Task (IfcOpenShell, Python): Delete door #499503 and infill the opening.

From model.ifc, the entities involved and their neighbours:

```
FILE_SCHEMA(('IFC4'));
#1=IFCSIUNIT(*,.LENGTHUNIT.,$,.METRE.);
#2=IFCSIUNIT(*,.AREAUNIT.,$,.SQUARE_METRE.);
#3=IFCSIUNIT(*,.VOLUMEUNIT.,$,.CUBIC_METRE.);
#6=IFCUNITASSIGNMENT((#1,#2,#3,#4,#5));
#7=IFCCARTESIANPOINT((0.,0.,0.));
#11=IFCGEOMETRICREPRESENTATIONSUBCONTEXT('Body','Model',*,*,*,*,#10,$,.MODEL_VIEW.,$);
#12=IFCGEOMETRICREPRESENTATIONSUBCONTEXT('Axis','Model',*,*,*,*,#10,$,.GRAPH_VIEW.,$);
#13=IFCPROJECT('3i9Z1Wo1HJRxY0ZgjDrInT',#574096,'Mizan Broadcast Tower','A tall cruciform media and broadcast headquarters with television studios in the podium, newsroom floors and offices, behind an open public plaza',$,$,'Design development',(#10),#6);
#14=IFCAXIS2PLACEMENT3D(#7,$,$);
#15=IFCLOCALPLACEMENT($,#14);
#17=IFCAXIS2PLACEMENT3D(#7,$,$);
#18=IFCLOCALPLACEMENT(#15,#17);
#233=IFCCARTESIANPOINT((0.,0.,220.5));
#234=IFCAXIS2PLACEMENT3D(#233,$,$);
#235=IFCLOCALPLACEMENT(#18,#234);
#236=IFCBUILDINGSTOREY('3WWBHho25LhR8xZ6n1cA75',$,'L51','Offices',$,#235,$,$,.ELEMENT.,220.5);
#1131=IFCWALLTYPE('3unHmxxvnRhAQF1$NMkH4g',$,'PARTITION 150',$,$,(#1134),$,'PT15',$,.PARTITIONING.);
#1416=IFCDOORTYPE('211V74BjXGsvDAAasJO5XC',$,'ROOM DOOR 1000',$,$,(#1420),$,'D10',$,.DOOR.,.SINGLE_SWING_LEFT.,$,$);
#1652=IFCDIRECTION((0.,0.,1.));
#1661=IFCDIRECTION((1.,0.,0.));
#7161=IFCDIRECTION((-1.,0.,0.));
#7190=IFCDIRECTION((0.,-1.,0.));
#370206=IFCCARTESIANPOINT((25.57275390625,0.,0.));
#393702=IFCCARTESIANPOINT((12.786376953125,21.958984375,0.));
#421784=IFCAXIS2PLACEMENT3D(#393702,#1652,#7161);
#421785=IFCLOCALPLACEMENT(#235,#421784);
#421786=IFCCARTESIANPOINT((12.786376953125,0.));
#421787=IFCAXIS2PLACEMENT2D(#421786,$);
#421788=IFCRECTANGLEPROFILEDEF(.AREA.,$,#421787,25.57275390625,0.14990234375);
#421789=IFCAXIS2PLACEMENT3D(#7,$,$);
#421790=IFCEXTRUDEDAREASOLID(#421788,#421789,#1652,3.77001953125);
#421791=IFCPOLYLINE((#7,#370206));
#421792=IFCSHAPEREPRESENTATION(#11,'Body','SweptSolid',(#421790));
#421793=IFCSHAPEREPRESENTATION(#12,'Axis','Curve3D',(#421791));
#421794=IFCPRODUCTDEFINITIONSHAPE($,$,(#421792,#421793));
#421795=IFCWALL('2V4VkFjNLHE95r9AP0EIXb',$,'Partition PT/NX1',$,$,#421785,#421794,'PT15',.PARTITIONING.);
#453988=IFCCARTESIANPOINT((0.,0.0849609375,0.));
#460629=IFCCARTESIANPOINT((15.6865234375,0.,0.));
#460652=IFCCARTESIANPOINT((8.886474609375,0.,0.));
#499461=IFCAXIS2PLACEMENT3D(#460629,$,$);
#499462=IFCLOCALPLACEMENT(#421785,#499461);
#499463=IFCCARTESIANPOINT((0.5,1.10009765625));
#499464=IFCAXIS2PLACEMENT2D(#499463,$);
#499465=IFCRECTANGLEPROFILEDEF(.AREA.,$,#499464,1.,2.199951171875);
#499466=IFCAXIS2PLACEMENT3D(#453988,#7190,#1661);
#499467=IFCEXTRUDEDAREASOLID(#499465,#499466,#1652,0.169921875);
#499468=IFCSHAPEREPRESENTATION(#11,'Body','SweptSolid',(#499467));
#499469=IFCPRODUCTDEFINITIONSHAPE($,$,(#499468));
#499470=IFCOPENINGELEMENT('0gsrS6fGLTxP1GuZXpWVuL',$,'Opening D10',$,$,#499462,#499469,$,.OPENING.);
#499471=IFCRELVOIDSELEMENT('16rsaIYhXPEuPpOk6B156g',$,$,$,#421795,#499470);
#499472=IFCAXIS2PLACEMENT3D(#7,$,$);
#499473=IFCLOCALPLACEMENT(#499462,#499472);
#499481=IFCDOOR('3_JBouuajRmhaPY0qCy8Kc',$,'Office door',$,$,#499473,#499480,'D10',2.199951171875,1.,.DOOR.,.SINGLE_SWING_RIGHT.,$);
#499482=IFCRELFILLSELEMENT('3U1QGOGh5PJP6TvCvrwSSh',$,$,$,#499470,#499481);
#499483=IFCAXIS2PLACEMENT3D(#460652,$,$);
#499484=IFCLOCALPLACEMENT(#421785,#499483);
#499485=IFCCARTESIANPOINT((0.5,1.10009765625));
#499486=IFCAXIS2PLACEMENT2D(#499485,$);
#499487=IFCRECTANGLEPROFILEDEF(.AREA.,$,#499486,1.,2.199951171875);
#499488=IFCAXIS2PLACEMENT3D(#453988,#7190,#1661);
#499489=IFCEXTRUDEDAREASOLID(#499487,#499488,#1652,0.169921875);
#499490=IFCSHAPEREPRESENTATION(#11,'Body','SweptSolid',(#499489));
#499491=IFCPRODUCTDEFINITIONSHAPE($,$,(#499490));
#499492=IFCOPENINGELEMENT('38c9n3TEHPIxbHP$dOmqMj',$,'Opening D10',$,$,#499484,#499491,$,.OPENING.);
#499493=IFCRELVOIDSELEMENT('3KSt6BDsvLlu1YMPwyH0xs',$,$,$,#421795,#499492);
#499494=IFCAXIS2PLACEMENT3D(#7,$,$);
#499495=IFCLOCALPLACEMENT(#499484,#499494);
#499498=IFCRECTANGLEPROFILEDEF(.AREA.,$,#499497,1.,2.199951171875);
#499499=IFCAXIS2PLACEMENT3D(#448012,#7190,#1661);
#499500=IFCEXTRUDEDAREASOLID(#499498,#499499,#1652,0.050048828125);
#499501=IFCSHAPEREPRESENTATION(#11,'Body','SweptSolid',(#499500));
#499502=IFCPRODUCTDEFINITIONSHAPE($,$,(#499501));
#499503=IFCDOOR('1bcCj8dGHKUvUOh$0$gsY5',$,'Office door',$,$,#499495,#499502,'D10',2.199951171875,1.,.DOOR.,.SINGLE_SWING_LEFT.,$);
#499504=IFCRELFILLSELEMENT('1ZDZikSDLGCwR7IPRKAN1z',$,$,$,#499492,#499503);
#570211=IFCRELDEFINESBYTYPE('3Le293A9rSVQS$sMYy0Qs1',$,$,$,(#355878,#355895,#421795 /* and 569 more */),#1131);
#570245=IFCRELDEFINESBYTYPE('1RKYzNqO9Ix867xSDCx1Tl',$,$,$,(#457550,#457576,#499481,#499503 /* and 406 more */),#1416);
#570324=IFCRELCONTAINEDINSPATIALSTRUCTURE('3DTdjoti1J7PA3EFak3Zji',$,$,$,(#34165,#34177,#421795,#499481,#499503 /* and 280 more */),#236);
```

```python
import ifcopenshell
import ifcopenshell.api.feature
import ifcopenshell.api.root
import ifcopenshell.geom
import ifcopenshell.util.shape

model = ifcopenshell.open("model.ifc")
settings = ifcopenshell.geom.settings()


def volume(element):
    """Net volume in cubic metres, openings subtracted."""
    shape = ifcopenshell.geom.create_shape(settings, element)
    return ifcopenshell.util.shape.get_volume(shape.geometry)


door = model.by_id(499503)
opening = door.FillsVoids[0].RelatingOpeningElement
wall = opening.VoidsElements[0].RelatingBuildingElement
before = volume(wall)

ifcopenshell.api.root.remove_product(model, product=door)
ifcopenshell.api.feature.remove_feature(model, feature=opening)

after = volume(wall)

print(f"wall volume {before:.3f} -> {after:.3f} m3")

model.write("model_edited.ifc")
```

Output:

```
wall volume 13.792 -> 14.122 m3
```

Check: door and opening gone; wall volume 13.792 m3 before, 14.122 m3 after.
